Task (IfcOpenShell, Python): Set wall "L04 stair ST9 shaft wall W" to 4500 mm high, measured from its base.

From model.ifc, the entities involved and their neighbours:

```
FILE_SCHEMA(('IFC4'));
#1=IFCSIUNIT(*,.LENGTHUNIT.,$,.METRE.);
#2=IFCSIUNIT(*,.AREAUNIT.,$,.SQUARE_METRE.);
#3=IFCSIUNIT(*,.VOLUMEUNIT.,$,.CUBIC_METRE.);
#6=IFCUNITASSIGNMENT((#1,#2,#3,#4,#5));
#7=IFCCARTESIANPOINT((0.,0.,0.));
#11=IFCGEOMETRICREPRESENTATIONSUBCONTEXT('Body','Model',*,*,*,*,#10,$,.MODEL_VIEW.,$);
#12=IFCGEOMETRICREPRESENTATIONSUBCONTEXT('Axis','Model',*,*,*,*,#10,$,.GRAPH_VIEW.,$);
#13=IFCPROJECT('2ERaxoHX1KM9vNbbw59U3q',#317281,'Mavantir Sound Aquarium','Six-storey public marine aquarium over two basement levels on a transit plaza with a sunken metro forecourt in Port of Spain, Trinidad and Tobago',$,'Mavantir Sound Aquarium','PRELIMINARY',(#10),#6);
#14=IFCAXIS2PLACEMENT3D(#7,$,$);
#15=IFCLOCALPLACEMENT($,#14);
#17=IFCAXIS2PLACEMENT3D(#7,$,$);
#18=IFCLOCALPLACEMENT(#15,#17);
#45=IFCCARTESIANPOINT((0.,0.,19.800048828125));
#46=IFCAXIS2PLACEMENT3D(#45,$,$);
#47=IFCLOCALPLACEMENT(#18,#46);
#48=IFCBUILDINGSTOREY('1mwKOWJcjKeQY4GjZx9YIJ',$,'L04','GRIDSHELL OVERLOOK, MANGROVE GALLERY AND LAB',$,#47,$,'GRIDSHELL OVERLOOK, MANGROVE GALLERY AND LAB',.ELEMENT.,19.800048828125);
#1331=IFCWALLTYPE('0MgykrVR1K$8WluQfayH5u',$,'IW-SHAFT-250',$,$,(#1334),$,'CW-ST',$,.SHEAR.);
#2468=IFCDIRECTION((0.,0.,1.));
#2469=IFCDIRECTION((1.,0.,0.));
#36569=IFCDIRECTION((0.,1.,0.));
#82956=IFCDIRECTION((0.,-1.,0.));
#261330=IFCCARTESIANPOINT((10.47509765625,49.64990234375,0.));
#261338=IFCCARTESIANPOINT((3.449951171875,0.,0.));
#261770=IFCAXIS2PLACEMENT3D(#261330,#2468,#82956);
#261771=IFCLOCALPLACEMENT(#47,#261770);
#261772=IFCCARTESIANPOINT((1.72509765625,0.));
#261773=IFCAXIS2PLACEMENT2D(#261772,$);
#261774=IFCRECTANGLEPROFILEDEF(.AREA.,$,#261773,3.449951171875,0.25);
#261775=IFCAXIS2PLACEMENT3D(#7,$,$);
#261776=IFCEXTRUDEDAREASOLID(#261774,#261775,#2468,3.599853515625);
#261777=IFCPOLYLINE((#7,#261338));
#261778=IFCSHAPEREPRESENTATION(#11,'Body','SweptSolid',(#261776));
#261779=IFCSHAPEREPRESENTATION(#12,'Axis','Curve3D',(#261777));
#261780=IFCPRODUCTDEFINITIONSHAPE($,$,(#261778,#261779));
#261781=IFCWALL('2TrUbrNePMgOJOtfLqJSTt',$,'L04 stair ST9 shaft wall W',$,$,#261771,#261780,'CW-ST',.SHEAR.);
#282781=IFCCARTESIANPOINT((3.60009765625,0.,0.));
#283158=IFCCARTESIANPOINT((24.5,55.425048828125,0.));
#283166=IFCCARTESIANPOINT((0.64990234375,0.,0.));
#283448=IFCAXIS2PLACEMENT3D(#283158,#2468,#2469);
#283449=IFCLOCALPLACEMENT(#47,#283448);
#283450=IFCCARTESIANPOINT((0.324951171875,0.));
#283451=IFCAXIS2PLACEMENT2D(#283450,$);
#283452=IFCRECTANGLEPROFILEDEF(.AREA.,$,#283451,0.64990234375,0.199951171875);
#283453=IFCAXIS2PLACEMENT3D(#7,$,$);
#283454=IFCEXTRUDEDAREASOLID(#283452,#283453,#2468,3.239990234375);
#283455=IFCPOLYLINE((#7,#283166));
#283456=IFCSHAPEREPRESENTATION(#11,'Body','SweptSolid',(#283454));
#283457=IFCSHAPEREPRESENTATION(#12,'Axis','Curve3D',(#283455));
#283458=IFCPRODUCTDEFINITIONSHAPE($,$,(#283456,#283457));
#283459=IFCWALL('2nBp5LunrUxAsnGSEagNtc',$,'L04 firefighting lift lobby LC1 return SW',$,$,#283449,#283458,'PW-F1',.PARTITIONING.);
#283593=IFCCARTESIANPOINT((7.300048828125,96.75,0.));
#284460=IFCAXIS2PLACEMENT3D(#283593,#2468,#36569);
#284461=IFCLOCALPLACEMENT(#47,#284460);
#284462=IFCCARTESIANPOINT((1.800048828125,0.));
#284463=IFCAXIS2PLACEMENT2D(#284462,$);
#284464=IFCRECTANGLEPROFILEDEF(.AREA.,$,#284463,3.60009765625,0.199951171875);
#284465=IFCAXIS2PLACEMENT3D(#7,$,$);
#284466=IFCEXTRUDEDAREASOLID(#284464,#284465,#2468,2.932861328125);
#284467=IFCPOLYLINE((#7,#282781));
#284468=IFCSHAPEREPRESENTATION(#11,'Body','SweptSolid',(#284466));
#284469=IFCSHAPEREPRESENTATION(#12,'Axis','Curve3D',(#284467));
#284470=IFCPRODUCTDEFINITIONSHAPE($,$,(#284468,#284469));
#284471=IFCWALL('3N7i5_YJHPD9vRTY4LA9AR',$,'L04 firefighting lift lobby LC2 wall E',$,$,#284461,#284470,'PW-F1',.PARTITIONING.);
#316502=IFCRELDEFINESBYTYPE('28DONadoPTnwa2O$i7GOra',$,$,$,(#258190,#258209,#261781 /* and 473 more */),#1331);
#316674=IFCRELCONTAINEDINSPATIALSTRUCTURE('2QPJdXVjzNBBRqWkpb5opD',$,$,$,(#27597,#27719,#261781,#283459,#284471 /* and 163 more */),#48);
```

```python
import ifcopenshell
import ifcopenshell.geom
import ifcopenshell.util.representation
import ifcopenshell.util.shape
import ifcopenshell.util.unit

model = ifcopenshell.open("model.ifc")
unit_scale = ifcopenshell.util.unit.calculate_unit_scale(model)
settings = ifcopenshell.geom.settings()


def volume(element):
    """Net volume in cubic metres, openings subtracted."""
    shape = ifcopenshell.geom.create_shape(settings, element)
    return ifcopenshell.util.shape.get_volume(shape.geometry)


wall = model.by_id(261781)
before = volume(wall)

body = ifcopenshell.util.representation.get_representation(wall, "Model", "Body")
solid = body.Items[0]
old_height = solid.Depth
solid.Depth = 4.5 / unit_scale
after = volume(wall)

print(f"height {old_height:g} -> {solid.Depth:g}, volume {before:.3f} -> {after:.3f} m3")

model.write("model_rev.ifc")
```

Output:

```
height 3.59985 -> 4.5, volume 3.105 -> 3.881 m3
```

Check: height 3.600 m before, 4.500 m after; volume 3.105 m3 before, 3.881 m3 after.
